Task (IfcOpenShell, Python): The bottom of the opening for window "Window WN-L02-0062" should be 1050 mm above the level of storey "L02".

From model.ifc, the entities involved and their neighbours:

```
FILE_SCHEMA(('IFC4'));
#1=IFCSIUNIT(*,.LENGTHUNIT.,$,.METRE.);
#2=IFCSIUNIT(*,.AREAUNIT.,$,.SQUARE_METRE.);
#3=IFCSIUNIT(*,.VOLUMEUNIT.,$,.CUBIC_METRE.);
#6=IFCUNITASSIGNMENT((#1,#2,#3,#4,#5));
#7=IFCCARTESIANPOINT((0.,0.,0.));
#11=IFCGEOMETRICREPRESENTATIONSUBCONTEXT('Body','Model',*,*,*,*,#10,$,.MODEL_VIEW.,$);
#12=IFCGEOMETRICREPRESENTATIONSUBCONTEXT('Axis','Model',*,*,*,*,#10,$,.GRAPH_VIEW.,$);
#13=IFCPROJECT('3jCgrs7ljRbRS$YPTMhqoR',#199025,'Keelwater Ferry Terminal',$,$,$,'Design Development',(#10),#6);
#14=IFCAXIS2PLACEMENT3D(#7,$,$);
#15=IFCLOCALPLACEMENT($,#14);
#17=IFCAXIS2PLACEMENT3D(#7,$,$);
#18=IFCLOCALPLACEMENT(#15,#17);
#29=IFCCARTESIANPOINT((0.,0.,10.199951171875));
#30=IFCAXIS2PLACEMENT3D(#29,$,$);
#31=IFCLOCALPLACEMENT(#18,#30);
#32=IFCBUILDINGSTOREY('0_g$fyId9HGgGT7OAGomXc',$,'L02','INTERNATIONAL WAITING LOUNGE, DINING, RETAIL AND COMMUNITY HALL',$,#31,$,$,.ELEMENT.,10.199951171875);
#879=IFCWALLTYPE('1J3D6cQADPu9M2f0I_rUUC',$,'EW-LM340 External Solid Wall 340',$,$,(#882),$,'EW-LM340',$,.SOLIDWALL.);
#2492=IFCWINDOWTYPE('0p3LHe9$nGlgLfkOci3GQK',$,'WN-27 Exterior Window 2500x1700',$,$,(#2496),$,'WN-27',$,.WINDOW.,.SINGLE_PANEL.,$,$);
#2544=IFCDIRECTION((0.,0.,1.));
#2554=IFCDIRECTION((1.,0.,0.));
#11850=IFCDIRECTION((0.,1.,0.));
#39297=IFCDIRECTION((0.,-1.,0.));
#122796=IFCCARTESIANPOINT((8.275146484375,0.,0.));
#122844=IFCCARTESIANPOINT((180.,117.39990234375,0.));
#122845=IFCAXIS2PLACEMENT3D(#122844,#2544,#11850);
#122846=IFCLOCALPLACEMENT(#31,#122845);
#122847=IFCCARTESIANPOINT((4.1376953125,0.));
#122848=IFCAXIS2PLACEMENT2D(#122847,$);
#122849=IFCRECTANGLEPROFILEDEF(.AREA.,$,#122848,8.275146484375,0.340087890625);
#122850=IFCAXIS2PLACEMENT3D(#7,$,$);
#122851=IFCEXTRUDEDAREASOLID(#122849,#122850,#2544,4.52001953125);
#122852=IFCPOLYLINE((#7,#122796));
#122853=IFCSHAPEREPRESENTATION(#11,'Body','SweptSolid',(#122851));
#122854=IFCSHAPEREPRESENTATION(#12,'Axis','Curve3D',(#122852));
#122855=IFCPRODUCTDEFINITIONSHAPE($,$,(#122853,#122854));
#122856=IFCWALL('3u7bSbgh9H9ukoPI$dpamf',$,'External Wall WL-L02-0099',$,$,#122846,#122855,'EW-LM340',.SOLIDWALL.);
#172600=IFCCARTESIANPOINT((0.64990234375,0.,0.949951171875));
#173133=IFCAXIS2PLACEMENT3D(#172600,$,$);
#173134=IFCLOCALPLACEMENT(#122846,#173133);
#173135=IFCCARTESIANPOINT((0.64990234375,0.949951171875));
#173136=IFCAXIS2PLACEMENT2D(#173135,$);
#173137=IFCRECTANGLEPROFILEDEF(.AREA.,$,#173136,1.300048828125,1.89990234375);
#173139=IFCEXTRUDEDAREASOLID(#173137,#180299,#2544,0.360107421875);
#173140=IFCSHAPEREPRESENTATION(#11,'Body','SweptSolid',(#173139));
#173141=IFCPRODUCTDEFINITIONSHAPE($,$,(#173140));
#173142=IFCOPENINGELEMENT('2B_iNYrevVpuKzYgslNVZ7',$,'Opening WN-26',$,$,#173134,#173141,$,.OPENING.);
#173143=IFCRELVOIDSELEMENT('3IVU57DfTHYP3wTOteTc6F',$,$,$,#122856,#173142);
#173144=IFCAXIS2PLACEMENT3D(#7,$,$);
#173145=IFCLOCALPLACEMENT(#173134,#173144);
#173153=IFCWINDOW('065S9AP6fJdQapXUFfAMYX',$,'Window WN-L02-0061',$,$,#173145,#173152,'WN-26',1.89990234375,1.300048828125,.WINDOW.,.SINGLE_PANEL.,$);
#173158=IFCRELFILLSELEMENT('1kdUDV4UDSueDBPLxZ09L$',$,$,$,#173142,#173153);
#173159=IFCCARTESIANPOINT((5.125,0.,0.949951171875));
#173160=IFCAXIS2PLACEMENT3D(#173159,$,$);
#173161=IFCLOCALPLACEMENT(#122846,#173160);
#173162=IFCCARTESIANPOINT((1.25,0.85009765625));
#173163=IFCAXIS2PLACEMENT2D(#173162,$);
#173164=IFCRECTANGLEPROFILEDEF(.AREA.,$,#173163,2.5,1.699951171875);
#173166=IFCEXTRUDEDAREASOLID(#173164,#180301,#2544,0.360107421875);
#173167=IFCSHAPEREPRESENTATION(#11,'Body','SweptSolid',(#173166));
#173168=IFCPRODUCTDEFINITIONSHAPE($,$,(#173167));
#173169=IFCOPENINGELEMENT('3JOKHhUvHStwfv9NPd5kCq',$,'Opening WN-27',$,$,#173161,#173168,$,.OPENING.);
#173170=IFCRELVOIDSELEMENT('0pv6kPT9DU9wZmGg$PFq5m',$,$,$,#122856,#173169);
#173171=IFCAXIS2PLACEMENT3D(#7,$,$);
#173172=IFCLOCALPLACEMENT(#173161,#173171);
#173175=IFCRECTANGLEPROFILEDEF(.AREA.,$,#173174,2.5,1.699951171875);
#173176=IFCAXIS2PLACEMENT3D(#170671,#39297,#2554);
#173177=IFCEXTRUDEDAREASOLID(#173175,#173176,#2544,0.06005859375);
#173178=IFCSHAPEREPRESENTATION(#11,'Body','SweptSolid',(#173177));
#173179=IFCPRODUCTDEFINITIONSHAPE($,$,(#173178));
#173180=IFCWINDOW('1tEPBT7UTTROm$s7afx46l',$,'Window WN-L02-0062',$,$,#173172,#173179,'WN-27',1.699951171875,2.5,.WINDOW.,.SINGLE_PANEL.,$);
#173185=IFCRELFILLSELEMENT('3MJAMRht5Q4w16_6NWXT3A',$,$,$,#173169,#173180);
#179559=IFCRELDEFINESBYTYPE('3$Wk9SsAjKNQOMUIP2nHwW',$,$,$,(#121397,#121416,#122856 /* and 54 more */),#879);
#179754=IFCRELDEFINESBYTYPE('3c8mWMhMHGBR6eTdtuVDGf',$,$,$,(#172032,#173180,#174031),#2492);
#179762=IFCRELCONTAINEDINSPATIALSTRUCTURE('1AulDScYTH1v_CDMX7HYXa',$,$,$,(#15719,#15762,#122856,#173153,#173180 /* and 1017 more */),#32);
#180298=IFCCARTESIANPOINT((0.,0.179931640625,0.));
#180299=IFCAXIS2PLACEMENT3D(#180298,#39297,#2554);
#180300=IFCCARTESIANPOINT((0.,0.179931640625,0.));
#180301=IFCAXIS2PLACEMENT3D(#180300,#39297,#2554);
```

```python
import numpy as np
import ifcopenshell
import ifcopenshell.api.geometry
import ifcopenshell.geom
import ifcopenshell.util.element
import ifcopenshell.util.placement
import ifcopenshell.util.shape
import ifcopenshell.util.unit

model = ifcopenshell.open("model.ifc")
unit_scale = ifcopenshell.util.unit.calculate_unit_scale(model)

window = model.by_guid("1tEPBT7UTTROm$s7afx46l")
opening = window.FillsVoids[0].RelatingOpeningElement
storey = ifcopenshell.util.element.get_container(window, ifc_class="IfcBuildingStorey")
level = ifcopenshell.util.placement.get_local_placement(storey.ObjectPlacement)[2, 3]

# The opening's origin need not be at the sill, so measure its lowest point.
shape = ifcopenshell.geom.create_shape(ifcopenshell.geom.settings(), opening)
bottom = ifcopenshell.util.shape.get_shape_bottom_elevation(shape, shape.geometry) / unit_scale
dz = level + 1.05 / unit_scale - bottom

shift = np.array([0.0, 0.0, dz])
# The window is placed relative to its opening, so it follows when the opening moves.
matrix = ifcopenshell.util.placement.get_local_placement(opening.ObjectPlacement)
matrix[:3, 3] += shift
ifcopenshell.api.geometry.edit_object_placement(
    model, product=opening, matrix=matrix, is_si=False, should_transform_children=True
)

print(f"moved by {dz * unit_scale:+.3f} m")

model.write("model_updated.ifc")
```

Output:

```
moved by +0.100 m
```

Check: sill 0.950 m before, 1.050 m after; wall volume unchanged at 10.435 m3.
